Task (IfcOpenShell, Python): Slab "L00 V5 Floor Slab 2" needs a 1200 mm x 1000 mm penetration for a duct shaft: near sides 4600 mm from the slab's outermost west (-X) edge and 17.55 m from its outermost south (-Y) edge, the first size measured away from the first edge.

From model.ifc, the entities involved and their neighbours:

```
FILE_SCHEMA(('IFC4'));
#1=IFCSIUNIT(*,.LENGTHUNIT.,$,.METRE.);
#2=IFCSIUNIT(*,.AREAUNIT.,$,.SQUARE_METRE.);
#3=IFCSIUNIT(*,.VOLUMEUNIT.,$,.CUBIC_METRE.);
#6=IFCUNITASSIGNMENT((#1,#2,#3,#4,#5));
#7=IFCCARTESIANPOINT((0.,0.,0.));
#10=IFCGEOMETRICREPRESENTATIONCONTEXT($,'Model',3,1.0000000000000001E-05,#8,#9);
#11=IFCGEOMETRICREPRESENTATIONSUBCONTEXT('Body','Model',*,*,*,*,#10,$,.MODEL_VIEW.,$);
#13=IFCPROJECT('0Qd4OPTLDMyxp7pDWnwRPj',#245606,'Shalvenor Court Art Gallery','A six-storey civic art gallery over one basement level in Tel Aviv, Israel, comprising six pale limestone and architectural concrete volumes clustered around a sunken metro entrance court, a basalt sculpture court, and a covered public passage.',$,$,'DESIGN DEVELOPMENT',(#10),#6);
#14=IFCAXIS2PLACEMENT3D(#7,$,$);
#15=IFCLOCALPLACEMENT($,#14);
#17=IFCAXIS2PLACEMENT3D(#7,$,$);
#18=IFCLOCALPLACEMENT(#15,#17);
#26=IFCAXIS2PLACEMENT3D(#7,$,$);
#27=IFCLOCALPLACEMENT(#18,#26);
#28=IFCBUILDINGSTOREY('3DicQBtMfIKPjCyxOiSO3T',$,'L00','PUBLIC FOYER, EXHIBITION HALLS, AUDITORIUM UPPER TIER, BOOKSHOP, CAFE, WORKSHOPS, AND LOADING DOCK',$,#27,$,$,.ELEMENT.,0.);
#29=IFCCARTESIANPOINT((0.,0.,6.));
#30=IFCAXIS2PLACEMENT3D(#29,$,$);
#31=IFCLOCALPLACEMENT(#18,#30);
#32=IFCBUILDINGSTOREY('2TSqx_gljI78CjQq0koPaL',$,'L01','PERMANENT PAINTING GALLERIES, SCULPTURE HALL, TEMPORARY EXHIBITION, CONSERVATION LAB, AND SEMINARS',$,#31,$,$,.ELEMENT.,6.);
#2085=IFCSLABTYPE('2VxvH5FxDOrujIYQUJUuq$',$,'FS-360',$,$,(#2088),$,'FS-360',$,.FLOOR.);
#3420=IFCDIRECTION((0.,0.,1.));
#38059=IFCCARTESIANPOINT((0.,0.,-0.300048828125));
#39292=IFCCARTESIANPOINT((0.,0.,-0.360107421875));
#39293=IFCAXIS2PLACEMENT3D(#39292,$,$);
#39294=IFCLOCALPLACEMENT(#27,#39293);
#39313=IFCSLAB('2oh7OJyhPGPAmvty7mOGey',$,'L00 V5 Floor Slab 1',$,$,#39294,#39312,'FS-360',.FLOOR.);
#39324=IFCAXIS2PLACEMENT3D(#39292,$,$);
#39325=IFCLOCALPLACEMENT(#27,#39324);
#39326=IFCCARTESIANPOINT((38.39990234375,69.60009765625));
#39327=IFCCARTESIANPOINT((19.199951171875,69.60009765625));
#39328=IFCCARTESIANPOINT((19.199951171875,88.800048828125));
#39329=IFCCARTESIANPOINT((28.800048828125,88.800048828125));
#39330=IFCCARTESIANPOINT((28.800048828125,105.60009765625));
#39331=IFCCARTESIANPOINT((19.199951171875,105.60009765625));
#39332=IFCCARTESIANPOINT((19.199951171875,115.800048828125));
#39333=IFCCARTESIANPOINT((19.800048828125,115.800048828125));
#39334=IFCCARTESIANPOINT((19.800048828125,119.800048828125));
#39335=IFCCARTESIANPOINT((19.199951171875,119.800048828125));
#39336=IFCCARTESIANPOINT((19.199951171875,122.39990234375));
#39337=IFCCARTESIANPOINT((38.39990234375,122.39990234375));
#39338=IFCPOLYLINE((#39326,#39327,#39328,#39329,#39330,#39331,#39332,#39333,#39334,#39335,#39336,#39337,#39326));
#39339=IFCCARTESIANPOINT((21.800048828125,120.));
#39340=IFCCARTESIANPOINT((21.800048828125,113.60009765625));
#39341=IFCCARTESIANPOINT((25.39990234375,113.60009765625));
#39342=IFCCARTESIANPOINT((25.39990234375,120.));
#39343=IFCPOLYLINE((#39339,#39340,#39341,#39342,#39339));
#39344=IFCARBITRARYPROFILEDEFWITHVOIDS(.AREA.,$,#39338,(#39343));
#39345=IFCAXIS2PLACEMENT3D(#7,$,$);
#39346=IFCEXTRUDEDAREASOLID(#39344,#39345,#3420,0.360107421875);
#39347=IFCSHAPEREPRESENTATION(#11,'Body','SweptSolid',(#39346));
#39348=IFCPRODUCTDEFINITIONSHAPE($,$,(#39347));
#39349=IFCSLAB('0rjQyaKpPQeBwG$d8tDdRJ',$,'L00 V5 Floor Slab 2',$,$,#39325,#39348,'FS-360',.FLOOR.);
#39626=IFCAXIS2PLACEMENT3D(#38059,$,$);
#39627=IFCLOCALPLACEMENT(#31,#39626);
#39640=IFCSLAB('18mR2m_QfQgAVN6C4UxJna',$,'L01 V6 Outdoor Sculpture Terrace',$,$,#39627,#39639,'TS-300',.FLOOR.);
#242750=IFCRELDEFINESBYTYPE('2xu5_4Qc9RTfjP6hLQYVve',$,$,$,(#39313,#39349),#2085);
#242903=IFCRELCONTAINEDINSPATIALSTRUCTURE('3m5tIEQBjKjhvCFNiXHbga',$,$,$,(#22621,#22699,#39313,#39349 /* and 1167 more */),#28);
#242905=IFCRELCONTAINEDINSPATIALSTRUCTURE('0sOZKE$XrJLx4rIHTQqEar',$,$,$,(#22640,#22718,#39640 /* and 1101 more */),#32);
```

```python
import numpy as np
import ifcopenshell
import ifcopenshell.api.feature
import ifcopenshell.api.geometry
import ifcopenshell.api.root
import ifcopenshell.geom
import ifcopenshell.util.placement
import ifcopenshell.util.representation
import ifcopenshell.util.shape
import ifcopenshell.util.unit

model = ifcopenshell.open("model.ifc")
unit_scale = ifcopenshell.util.unit.calculate_unit_scale(model)
settings = ifcopenshell.geom.settings()


def volume(element):
    """Net volume in cubic metres, openings subtracted."""
    shape = ifcopenshell.geom.create_shape(settings, element)
    return ifcopenshell.util.shape.get_volume(shape.geometry)


slab = model.by_id(39349)
before = volume(slab)

# Extent in the slab's own axes, in metres. The edges named are its -X and -Y sides.
slab_shape = ifcopenshell.geom.create_shape(settings, slab)
vertices = ifcopenshell.util.shape.get_vertices(slab_shape.geometry)
x_min, y_min, bottom = vertices.min(axis=0)
top = vertices[:, 2].max()

opening = ifcopenshell.api.root.create_entity(model, ifc_class="IfcOpeningElement", name="Duct shaft opening", predefined_type="OPENING")
context = ifcopenshell.util.representation.get_context(model, "Model", "Body", "MODEL_VIEW")
width, depth = 1.2, 1
outline = [(0.0, 0.0), (width, 0.0), (width, depth), (0.0, depth), (0.0, 0.0)]
# Overshoot both faces by 50 mm so the cut is clean.
shape = ifcopenshell.api.geometry.add_slab_representation(
    model, context=context, depth=top - bottom + 0.1, polyline=outline
)
ifcopenshell.api.geometry.assign_representation(model, product=opening, representation=shape)

matrix = ifcopenshell.util.placement.get_local_placement(slab.ObjectPlacement)
matrix[:, 3] = matrix @ np.append(np.array([x_min + 4.6, y_min + 17.55, bottom - 0.05]) / unit_scale, 1.0)
ifcopenshell.api.geometry.edit_object_placement(model, product=opening, matrix=matrix, is_si=False)
ifcopenshell.api.feature.add_feature(model, feature=opening, element=slab)

after = volume(slab)

print(f"slab volume {before:.3f} -> {after:.3f} m3")

model.write("model_updated.ifc")
```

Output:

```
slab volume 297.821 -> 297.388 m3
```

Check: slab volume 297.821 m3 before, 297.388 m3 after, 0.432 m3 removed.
